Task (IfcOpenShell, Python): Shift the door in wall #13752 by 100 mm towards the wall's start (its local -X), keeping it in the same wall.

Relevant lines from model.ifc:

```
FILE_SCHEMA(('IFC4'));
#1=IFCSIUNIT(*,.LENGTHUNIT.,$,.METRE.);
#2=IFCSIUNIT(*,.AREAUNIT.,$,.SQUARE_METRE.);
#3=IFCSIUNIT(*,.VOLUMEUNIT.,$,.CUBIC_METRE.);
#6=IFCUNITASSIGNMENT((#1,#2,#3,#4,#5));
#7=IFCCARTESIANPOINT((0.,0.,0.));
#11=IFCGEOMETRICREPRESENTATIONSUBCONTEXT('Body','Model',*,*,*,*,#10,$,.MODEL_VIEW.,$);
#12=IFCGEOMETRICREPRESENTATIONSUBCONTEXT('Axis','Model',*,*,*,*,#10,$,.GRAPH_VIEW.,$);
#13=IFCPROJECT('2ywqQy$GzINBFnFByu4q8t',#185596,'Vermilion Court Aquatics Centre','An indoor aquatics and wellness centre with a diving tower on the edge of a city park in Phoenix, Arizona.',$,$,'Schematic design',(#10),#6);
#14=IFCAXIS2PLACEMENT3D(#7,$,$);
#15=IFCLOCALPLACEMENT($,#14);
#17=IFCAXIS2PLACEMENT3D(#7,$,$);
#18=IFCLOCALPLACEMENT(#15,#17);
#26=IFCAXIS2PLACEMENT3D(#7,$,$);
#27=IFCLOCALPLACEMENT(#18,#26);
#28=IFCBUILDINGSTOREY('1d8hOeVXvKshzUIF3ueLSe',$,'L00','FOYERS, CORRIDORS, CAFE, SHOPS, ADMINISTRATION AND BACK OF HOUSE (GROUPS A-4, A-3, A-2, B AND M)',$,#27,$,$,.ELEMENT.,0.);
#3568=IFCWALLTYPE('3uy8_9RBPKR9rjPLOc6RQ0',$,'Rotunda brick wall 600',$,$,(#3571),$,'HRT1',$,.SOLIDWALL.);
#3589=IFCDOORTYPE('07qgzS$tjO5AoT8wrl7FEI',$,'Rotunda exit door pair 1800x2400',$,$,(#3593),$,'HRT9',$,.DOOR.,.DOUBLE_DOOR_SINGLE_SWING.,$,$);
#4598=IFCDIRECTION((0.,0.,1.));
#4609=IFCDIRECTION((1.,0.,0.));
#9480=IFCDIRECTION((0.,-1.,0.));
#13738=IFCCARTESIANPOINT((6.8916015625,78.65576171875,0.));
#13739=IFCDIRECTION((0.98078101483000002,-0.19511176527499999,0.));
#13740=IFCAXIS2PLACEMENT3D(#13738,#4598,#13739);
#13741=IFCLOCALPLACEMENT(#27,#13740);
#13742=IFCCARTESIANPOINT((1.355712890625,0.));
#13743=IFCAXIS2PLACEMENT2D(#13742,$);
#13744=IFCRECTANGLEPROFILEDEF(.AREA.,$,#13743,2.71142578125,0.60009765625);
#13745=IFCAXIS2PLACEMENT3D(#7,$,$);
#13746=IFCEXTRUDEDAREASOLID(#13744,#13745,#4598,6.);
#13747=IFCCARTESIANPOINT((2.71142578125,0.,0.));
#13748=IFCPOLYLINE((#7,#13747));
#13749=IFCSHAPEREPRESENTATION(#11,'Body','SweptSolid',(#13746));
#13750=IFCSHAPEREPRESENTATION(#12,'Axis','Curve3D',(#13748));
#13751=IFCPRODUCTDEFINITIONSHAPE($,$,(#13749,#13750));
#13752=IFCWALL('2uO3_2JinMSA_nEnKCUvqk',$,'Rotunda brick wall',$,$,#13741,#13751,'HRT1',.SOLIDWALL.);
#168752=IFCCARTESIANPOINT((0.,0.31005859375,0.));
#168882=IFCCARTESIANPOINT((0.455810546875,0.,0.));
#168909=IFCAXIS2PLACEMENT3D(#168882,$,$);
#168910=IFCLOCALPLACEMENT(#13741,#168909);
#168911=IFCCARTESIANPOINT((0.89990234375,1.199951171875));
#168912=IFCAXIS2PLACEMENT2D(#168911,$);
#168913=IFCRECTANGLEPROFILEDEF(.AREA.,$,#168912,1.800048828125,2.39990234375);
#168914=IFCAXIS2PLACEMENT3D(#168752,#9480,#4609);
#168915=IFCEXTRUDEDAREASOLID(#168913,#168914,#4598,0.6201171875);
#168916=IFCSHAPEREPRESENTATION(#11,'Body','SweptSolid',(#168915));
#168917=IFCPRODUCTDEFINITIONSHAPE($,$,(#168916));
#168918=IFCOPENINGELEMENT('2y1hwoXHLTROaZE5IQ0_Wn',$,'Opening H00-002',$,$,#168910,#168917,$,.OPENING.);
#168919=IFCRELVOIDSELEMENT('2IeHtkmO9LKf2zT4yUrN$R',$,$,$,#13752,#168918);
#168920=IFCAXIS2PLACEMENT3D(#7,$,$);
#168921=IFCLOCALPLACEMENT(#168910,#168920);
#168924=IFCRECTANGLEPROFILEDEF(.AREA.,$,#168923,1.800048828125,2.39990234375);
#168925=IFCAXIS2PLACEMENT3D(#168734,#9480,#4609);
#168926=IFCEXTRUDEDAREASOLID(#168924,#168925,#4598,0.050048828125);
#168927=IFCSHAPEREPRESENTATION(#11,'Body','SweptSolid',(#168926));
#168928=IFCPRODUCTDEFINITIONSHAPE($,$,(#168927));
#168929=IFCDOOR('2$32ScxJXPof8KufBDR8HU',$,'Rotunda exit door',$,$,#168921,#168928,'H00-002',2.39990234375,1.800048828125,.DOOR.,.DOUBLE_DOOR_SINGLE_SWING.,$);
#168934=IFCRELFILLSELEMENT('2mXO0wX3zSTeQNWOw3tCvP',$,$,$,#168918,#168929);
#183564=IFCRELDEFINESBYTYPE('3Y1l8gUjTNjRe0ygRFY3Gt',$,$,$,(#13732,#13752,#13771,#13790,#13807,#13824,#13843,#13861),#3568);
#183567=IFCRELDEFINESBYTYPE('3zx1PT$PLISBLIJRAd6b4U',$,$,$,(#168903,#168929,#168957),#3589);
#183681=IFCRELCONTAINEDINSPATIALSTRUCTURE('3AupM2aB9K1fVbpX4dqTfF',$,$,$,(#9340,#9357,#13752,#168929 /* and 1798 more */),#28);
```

```python
import ifcopenshell
import ifcopenshell.api.geometry
import ifcopenshell.util.placement

model = ifcopenshell.open("model.ifc")

door = model.by_id(168929)
opening = door.FillsVoids[0].RelatingOpeningElement
wall = opening.VoidsElements[0].RelatingBuildingElement

wall_matrix = ifcopenshell.util.placement.get_local_placement(wall.ObjectPlacement)
shift = wall_matrix[:3, 0] * -0.1
before = ifcopenshell.util.placement.get_local_placement(door.ObjectPlacement)[:3, 3].copy()

# The door is placed relative to its opening, so it follows when the opening moves.
matrix = ifcopenshell.util.placement.get_local_placement(opening.ObjectPlacement)
matrix[:3, 3] += shift
ifcopenshell.api.geometry.edit_object_placement(
    model, product=opening, matrix=matrix, is_si=False, should_transform_children=True
)

after = ifcopenshell.util.placement.get_local_placement(door.ObjectPlacement)[:3, 3]
print("door moved by", (after - before).round(3) + 0.0)

model.write("model-out.ifc")
```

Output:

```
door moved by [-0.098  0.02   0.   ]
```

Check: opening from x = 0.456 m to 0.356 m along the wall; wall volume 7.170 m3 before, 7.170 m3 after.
